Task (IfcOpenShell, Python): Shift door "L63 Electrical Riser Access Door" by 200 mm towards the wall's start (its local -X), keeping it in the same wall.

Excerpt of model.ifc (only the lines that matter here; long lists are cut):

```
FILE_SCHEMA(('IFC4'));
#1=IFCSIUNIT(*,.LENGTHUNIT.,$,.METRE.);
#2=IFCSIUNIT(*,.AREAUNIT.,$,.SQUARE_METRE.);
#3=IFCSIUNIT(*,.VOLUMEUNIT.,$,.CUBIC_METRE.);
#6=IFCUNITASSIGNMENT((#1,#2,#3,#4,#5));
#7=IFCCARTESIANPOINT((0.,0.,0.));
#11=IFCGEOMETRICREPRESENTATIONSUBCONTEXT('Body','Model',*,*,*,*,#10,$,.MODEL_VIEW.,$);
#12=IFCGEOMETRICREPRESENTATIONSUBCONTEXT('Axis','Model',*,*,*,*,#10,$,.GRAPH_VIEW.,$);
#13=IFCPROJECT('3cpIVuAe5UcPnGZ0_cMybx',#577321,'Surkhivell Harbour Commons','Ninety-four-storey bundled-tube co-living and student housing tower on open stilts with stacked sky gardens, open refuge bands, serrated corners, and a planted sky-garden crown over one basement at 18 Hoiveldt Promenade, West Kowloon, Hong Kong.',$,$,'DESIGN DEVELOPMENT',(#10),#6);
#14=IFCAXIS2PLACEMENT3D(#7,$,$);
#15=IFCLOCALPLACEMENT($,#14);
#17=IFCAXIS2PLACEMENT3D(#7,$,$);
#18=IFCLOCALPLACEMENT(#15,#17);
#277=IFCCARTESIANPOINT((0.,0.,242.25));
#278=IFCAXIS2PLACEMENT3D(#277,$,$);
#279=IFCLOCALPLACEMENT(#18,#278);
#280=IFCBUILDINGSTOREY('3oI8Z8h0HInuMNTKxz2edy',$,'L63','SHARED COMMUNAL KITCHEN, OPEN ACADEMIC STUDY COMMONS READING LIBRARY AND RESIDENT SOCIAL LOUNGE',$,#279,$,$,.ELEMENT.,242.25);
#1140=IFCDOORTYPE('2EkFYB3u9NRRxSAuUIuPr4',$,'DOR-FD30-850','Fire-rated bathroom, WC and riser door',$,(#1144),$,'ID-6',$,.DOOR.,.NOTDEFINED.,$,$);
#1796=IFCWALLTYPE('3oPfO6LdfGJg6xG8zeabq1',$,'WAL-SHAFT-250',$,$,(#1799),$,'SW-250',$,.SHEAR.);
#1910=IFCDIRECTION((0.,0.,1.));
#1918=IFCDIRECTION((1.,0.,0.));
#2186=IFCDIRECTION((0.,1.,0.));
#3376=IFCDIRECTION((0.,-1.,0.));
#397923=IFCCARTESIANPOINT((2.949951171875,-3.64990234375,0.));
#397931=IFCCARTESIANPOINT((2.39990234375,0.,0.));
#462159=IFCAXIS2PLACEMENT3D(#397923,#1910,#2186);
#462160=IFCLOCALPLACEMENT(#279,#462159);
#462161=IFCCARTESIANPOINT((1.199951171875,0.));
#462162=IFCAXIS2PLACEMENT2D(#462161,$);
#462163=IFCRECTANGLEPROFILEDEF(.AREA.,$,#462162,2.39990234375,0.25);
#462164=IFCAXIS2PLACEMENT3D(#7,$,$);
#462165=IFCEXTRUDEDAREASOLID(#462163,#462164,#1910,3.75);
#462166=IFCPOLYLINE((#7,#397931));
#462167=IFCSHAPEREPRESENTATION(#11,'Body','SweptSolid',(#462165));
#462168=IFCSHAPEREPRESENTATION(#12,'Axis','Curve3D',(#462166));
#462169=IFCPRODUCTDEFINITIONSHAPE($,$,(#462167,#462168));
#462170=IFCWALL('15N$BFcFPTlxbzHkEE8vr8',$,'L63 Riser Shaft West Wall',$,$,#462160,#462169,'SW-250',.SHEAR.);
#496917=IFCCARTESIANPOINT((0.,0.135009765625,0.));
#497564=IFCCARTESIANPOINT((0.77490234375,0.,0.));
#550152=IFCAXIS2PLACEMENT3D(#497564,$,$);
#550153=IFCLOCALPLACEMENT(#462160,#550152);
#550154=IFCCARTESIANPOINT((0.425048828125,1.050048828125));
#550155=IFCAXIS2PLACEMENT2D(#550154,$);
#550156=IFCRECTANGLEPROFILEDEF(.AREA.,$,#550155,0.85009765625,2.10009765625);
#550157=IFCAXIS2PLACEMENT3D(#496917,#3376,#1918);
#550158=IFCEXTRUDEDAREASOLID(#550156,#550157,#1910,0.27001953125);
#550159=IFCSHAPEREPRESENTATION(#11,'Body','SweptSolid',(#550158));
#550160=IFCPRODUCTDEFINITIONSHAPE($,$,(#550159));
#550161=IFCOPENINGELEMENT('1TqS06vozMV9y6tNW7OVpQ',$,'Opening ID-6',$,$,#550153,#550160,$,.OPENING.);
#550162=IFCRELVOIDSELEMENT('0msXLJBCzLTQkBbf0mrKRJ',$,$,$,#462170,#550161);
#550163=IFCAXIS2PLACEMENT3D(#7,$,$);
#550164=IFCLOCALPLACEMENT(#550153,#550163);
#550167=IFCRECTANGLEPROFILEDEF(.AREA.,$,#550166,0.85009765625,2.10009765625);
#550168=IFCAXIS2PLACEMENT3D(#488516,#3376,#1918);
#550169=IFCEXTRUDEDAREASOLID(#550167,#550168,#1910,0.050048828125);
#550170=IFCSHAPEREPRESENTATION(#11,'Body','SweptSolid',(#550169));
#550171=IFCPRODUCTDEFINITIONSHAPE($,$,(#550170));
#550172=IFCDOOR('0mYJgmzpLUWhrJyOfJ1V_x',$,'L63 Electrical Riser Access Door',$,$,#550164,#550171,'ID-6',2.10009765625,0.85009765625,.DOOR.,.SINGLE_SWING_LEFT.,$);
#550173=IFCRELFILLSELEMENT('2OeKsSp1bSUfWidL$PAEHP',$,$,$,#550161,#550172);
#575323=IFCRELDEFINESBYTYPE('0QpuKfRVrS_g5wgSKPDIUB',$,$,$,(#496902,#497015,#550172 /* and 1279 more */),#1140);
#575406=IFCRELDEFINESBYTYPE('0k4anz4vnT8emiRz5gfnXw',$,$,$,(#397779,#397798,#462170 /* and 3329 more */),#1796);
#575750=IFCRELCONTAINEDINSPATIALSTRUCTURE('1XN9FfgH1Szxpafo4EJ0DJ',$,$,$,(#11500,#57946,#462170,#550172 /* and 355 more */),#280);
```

```python
import ifcopenshell
import ifcopenshell.api.geometry
import ifcopenshell.util.placement
import ifcopenshell.util.unit

model = ifcopenshell.open("model.ifc")
unit_scale = ifcopenshell.util.unit.calculate_unit_scale(model)

door = model.by_guid("0mYJgmzpLUWhrJyOfJ1V_x")
opening = door.FillsVoids[0].RelatingOpeningElement
wall = opening.VoidsElements[0].RelatingBuildingElement

wall_matrix = ifcopenshell.util.placement.get_local_placement(wall.ObjectPlacement)
shift = wall_matrix[:3, 0] * -0.2 / unit_scale
before = ifcopenshell.util.placement.get_local_placement(door.ObjectPlacement)[:3, 3].copy()

# The door is placed relative to its opening, so it follows when the opening moves.
matrix = ifcopenshell.util.placement.get_local_placement(opening.ObjectPlacement)
matrix[:3, 3] += shift
ifcopenshell.api.geometry.edit_object_placement(
    model, product=opening, matrix=matrix, is_si=False, should_transform_children=True
)

after = ifcopenshell.util.placement.get_local_placement(door.ObjectPlacement)[:3, 3]
print("door moved by", (after - before).round(3) + 0.0)

model.write("model_updated.ifc")
```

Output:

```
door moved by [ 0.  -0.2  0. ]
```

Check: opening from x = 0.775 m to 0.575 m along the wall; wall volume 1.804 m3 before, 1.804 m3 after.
